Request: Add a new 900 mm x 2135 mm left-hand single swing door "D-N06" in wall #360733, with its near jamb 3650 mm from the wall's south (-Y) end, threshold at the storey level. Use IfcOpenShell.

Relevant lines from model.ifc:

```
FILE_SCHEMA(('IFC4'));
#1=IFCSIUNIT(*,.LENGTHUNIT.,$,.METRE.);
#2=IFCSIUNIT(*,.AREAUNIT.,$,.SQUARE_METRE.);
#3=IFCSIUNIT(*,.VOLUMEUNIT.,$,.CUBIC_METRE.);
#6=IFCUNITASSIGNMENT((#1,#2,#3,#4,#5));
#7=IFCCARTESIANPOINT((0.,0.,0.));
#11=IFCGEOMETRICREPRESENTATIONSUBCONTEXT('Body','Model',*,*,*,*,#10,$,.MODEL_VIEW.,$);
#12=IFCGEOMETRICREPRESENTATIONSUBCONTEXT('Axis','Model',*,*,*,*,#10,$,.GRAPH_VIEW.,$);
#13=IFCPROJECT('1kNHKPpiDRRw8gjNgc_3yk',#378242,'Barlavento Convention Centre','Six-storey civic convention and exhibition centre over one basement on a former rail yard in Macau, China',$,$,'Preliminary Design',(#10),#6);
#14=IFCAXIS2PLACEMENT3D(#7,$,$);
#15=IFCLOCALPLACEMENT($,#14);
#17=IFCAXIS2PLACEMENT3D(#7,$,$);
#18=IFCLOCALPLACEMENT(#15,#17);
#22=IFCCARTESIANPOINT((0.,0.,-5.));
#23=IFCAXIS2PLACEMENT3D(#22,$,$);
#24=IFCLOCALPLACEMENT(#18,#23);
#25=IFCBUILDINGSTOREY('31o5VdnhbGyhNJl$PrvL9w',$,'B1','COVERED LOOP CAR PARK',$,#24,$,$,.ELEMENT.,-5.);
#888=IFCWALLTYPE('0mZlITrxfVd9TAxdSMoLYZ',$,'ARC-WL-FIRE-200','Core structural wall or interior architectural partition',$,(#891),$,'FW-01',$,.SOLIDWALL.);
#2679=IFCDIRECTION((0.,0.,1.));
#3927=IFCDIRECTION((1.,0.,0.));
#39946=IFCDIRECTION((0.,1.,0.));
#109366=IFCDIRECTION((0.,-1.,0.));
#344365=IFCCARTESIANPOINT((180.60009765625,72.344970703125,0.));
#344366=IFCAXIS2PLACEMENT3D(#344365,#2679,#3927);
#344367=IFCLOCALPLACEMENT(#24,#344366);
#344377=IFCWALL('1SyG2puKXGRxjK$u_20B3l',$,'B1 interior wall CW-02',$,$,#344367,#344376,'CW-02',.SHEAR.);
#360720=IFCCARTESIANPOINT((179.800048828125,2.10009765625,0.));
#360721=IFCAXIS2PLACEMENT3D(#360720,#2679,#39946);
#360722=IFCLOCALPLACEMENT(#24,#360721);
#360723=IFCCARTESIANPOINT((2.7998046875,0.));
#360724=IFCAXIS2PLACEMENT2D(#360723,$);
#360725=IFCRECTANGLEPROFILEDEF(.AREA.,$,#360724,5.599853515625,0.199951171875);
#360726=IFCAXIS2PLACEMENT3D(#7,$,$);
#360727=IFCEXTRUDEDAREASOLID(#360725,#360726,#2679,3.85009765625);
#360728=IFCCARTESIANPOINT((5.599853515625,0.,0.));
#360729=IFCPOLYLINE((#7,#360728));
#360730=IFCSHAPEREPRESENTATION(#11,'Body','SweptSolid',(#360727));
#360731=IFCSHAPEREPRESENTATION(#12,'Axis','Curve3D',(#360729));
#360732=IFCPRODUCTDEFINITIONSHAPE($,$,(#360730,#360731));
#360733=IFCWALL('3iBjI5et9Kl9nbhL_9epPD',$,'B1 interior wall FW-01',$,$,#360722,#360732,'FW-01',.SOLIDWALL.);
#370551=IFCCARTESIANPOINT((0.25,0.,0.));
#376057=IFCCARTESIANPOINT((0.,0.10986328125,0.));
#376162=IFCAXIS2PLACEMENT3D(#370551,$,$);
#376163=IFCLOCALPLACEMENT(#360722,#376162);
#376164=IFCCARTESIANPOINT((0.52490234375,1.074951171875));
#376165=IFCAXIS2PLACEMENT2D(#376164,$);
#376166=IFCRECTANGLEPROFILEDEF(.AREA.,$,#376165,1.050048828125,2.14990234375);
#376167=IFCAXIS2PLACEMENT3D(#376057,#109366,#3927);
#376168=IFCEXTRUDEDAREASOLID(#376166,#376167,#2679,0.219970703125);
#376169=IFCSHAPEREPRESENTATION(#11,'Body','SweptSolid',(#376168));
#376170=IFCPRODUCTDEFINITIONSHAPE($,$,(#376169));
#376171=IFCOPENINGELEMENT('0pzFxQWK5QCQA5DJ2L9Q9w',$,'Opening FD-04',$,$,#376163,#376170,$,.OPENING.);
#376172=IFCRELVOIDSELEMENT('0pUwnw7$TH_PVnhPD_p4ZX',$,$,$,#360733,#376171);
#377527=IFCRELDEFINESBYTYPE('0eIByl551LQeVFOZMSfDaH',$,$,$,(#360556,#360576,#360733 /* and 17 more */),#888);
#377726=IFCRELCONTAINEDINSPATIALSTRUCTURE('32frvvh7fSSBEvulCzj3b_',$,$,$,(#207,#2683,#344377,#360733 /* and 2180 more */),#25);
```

```python
import numpy as np
import ifcopenshell
import ifcopenshell.api.feature
import ifcopenshell.api.geometry
import ifcopenshell.api.root
import ifcopenshell.api.spatial
import ifcopenshell.geom
import ifcopenshell.util.element
import ifcopenshell.util.placement
import ifcopenshell.util.representation
import ifcopenshell.util.shape
import ifcopenshell.util.unit

model = ifcopenshell.open("model.ifc")
unit_scale = ifcopenshell.util.unit.calculate_unit_scale(model)
settings = ifcopenshell.geom.settings()


def volume(element):
    """Net volume in cubic metres, openings subtracted."""
    shape = ifcopenshell.geom.create_shape(settings, element)
    return ifcopenshell.util.shape.get_volume(shape.geometry)


wall = model.by_guid("3iBjI5et9Kl9nbhL_9epPD")
storey = ifcopenshell.util.element.get_container(wall, ifc_class="IfcBuildingStorey")
context = ifcopenshell.util.representation.get_context(model, "Model", "Body", "MODEL_VIEW")
before = volume(wall)

width, height, from_end, sill = 0.9, 2.135, 3.65, 0.0  # metres

# The wall runs along its own X axis, and the end named is its -X end.
wall_shape = ifcopenshell.geom.create_shape(settings, wall)
x, y, z = ifcopenshell.util.shape.get_vertices(wall_shape.geometry).T
start = x.min() + from_end
face, thickness = float(y.min()), float(y.max() - y.min())
wall_matrix = ifcopenshell.util.placement.get_local_placement(wall.ObjectPlacement)
level = ifcopenshell.util.placement.get_local_placement(storey.ObjectPlacement)[2, 3]


def in_wall(x, y):
    """Placement at x, y metres in the wall's axes, at sill height."""
    matrix = wall_matrix.copy()
    matrix[:, 3] = wall_matrix @ np.array([x / unit_scale, y / unit_scale, 0.0, 1.0])
    matrix[2, 3] = level + sill / unit_scale
    return matrix


# Opening: a box that overshoots both wall faces by 50 mm.
opening = ifcopenshell.api.root.create_entity(model, ifc_class="IfcOpeningElement", predefined_type="OPENING")
box = ifcopenshell.api.geometry.add_wall_representation(
    model, context=context, length=width, height=height, thickness=thickness + 0.1
)
ifcopenshell.api.geometry.assign_representation(model, product=opening, representation=box)
ifcopenshell.api.geometry.edit_object_placement(model, product=opening, matrix=in_wall(start, face - 0.05), is_si=False)
ifcopenshell.api.feature.add_feature(model, feature=opening, element=wall)

door = ifcopenshell.api.root.create_entity(model, ifc_class="IfcDoor", name="D-N06", predefined_type="DOOR")
door.OverallWidth, door.OverallHeight = width / unit_scale, height / unit_scale
door.OperationType = "SINGLE_SWING_LEFT"
body = ifcopenshell.api.geometry.add_door_representation(
    model,
    context=context,
    overall_width=door.OverallWidth,
    overall_height=door.OverallHeight,
    operation_type="SINGLE_SWING_LEFT",
    lining_properties={"LiningDepth": thickness / unit_scale, "ThresholdDepth": thickness / unit_scale},
)
ifcopenshell.api.geometry.assign_representation(model, product=door, representation=body)
ifcopenshell.api.spatial.assign_container(model, products=[door], relating_structure=storey)
ifcopenshell.api.feature.add_filling(model, opening=opening, element=door)

# The lining spans the wall, so the door starts at the wall face.
ifcopenshell.api.geometry.edit_object_placement(model, product=door, matrix=in_wall(start, face), is_si=False)

after = volume(wall)

print(f"wall volume {before:.3f} -> {after:.3f} m3")

model.write("model_updated.ifc")
```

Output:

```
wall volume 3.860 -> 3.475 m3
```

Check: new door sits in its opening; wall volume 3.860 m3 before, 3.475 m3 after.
